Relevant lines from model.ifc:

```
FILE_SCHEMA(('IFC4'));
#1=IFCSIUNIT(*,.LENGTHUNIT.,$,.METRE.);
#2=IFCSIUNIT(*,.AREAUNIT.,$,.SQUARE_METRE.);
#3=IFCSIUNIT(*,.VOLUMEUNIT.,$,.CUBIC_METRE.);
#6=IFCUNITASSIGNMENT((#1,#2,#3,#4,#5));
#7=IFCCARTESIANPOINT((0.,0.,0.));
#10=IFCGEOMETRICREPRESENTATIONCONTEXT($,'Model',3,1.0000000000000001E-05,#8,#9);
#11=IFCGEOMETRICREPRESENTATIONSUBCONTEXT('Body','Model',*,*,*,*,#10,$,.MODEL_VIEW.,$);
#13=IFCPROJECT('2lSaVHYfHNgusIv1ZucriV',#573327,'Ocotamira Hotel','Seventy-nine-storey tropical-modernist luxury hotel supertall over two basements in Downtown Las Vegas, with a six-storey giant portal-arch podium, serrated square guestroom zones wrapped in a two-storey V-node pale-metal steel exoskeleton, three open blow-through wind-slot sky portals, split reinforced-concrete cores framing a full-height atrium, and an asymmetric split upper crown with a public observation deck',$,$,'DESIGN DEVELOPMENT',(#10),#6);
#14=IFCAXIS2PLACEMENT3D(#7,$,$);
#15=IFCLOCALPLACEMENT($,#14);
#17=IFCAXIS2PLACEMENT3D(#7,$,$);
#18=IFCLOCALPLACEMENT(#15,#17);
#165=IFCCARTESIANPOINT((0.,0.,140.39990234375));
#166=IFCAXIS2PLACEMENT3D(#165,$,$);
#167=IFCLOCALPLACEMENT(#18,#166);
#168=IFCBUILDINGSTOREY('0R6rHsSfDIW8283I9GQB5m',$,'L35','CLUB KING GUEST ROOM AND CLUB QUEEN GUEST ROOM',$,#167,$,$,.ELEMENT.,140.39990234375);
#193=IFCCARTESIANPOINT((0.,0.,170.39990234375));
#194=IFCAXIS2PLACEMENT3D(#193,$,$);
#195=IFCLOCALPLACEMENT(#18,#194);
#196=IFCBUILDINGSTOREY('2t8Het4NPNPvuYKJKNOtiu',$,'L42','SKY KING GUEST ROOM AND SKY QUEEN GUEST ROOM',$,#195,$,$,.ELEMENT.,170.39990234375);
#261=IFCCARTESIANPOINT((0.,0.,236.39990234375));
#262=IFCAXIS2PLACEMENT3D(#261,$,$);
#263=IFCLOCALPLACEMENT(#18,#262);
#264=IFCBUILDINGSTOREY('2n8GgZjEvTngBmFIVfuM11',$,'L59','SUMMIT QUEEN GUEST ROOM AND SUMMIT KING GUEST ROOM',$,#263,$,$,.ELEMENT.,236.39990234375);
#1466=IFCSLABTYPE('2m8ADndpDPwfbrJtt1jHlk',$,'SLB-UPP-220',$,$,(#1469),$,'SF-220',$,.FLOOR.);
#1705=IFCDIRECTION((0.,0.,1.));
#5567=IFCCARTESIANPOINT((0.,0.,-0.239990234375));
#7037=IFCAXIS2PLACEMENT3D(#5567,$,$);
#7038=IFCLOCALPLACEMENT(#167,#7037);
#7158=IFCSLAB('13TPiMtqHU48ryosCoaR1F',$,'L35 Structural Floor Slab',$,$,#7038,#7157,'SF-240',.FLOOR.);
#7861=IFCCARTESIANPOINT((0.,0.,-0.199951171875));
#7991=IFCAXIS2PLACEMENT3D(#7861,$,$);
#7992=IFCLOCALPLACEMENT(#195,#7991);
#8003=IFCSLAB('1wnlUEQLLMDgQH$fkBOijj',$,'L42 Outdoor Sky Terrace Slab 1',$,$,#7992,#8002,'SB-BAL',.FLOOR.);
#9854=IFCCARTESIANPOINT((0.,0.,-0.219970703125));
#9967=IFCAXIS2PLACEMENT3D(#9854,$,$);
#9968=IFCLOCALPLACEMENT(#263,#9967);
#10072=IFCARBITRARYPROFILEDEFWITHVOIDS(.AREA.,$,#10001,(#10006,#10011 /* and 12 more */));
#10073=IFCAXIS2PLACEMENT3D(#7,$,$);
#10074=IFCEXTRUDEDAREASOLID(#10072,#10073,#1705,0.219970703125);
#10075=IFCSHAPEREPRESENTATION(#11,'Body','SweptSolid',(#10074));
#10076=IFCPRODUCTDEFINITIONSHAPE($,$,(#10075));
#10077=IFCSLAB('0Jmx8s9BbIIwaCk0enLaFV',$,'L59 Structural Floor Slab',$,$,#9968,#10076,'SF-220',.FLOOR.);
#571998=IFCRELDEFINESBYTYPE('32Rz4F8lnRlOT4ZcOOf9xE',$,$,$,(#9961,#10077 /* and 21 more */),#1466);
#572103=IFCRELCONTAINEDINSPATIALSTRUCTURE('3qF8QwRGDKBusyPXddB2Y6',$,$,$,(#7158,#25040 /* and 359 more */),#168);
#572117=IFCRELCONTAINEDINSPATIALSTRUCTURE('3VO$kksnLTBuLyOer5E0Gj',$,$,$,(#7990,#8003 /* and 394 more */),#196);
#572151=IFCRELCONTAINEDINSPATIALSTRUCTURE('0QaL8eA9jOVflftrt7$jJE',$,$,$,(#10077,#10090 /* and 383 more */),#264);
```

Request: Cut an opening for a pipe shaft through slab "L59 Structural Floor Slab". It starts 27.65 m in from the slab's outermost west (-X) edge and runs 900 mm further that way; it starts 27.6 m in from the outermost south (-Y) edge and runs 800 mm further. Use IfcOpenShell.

```python
import numpy as np
import ifcopenshell
import ifcopenshell.api.feature
import ifcopenshell.api.geometry
import ifcopenshell.api.root
import ifcopenshell.geom
import ifcopenshell.util.placement
import ifcopenshell.util.representation
import ifcopenshell.util.shape
import ifcopenshell.util.unit

model = ifcopenshell.open("model.ifc")
unit_scale = ifcopenshell.util.unit.calculate_unit_scale(model)
settings = ifcopenshell.geom.settings()


def volume(element):
    """Net volume in cubic metres, openings subtracted."""
    shape = ifcopenshell.geom.create_shape(settings, element)
    return ifcopenshell.util.shape.get_volume(shape.geometry)


slab = model.by_guid("0Jmx8s9BbIIwaCk0enLaFV")
before = volume(slab)

# Extent in the slab's own axes, in metres. The edges named are its -X and -Y sides.
slab_shape = ifcopenshell.geom.create_shape(settings, slab)
vertices = ifcopenshell.util.shape.get_vertices(slab_shape.geometry)
x_min, y_min, bottom = vertices.min(axis=0)
top = vertices[:, 2].max()

opening = ifcopenshell.api.root.create_entity(model, ifc_class="IfcOpeningElement", name="Pipe shaft opening", predefined_type="OPENING")
context = ifcopenshell.util.representation.get_context(model, "Model", "Body", "MODEL_VIEW")
width, depth = 0.9, 0.8
outline = [(0.0, 0.0), (width, 0.0), (width, depth), (0.0, depth), (0.0, 0.0)]
# Overshoot both faces by 50 mm so the cut is clean.
shape = ifcopenshell.api.geometry.add_slab_representation(
    model, context=context, depth=top - bottom + 0.1, polyline=outline
)
ifcopenshell.api.geometry.assign_representation(model, product=opening, representation=shape)

matrix = ifcopenshell.util.placement.get_local_placement(slab.ObjectPlacement)
matrix[:, 3] = matrix @ np.append(np.array([x_min + 27.65, y_min + 27.6, bottom - 0.05]) / unit_scale, 1.0)
ifcopenshell.api.geometry.edit_object_placement(model, product=opening, matrix=matrix, is_si=False)
ifcopenshell.api.feature.add_feature(model, feature=opening, element=slab)

after = volume(slab)

print(f"slab volume {before:.3f} -> {after:.3f} m3")

model.write("model_updated.ifc")
```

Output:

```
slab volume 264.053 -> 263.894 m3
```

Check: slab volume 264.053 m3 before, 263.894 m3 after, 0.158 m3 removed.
